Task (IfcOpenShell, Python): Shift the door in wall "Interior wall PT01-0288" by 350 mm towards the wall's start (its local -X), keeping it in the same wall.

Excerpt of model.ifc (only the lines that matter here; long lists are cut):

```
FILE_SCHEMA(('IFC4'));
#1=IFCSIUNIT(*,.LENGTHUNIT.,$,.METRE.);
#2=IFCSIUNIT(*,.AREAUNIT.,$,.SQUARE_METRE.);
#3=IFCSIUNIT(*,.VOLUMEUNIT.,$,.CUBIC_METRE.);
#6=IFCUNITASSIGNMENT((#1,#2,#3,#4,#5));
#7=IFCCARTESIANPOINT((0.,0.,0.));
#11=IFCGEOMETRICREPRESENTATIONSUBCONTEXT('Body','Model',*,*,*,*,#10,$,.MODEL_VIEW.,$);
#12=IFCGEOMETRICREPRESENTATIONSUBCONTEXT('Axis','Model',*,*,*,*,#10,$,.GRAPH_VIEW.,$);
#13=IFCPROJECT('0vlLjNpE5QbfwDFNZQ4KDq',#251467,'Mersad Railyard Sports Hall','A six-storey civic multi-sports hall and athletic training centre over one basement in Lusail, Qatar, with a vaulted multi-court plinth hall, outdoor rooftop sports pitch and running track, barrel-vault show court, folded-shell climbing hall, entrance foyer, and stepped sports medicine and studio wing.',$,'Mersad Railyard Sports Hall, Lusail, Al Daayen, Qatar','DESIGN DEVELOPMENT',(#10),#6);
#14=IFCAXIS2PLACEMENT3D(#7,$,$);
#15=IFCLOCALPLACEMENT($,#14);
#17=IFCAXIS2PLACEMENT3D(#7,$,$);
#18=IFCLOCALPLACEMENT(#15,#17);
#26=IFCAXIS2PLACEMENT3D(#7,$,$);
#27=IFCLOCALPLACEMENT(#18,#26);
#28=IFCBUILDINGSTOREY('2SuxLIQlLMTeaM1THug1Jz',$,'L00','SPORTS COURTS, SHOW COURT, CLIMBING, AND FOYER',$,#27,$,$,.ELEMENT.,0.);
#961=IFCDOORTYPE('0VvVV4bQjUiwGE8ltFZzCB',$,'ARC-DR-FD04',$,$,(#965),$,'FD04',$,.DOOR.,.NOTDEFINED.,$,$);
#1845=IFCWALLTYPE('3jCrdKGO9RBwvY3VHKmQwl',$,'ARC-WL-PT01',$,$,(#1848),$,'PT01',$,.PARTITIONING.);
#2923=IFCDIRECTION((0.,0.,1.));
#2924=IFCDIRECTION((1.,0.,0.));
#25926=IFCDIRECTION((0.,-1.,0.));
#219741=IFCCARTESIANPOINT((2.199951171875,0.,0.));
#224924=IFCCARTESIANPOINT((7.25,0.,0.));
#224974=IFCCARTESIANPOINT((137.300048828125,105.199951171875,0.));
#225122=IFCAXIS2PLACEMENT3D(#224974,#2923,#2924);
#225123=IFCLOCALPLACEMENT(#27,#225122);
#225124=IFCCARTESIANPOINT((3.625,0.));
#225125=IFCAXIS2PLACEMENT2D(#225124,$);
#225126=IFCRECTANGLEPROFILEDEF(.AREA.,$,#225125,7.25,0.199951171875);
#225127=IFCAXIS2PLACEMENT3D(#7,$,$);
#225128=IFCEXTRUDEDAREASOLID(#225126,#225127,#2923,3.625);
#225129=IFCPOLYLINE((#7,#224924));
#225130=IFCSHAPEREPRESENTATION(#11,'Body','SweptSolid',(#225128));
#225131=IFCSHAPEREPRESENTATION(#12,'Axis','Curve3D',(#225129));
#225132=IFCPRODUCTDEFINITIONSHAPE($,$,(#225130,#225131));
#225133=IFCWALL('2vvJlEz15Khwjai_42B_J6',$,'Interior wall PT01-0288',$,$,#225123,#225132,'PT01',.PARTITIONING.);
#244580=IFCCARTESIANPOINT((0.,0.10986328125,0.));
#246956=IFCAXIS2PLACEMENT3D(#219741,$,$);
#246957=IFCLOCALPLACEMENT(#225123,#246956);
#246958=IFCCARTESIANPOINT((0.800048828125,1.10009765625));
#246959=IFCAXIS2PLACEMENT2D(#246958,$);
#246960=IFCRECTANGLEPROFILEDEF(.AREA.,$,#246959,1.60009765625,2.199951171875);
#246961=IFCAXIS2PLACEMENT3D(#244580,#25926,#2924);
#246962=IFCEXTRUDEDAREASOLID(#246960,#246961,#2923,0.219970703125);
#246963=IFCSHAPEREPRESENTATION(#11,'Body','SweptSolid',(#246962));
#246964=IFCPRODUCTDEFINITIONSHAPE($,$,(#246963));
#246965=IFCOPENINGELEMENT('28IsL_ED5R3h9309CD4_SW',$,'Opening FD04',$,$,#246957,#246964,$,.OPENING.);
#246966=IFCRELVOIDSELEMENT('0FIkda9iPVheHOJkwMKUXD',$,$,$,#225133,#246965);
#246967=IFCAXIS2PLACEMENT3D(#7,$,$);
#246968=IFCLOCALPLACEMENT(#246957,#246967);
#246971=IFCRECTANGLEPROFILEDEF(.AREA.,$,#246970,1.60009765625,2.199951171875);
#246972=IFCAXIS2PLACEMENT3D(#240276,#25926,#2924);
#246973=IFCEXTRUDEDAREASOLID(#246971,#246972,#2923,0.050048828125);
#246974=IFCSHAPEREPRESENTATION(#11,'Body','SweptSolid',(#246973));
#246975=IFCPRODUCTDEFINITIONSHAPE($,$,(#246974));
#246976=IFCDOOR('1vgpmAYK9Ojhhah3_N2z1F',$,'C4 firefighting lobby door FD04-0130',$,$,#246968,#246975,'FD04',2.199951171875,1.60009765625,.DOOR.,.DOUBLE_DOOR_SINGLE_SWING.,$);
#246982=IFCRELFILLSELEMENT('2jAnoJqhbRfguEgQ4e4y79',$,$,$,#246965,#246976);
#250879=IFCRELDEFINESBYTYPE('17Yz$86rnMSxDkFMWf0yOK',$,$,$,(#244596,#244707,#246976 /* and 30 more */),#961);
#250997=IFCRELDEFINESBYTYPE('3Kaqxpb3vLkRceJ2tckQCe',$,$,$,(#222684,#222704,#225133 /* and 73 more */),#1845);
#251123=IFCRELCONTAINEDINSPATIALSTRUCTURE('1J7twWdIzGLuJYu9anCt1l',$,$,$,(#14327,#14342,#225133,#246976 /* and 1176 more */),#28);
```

```python
import ifcopenshell
import ifcopenshell.api.geometry
import ifcopenshell.util.placement

model = ifcopenshell.open("model.ifc")

door = model.by_guid("1vgpmAYK9Ojhhah3_N2z1F")
opening = door.FillsVoids[0].RelatingOpeningElement
wall = opening.VoidsElements[0].RelatingBuildingElement

wall_matrix = ifcopenshell.util.placement.get_local_placement(wall.ObjectPlacement)
shift = wall_matrix[:3, 0] * -0.35
before = ifcopenshell.util.placement.get_local_placement(door.ObjectPlacement)[:3, 3].copy()

# The door is placed relative to its opening, so it follows when the opening moves.
matrix = ifcopenshell.util.placement.get_local_placement(opening.ObjectPlacement)
matrix[:3, 3] += shift
ifcopenshell.api.geometry.edit_object_placement(
    model, product=opening, matrix=matrix, is_si=False, should_transform_children=True
)

after = ifcopenshell.util.placement.get_local_placement(door.ObjectPlacement)[:3, 3]
print("door moved by", (after - before).round(3) + 0.0)

model.write("model_rev.ifc")
```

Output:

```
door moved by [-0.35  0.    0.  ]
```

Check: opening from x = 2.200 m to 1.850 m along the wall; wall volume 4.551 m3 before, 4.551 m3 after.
